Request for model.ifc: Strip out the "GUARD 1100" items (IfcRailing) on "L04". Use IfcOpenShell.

First a look at what the model holds.

```python
import ifcopenshell
import ifcopenshell.util.element

model = ifcopenshell.open("model.ifc")
print(model.schema)
storey = next(s for s in model.by_type("IfcBuildingStorey") if s.Name == "L04")
railings = [e for e in ifcopenshell.util.element.get_decomposition(storey) if e.is_a("IfcRailing")]
seen = {}
for e in railings:
    element_type = ifcopenshell.util.element.get_type(e)
    name = element_type.Name if element_type not in (None, e) else None
    seen[name] = seen.get(name, 0) + 1
for name, count in sorted(seen.items(), key=str):
    print(count, "x", name)
```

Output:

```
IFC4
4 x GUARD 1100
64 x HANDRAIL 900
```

```python
import ifcopenshell
import ifcopenshell.api.root
import ifcopenshell.util.element

model = ifcopenshell.open("model.ifc")

storey = next(s for s in model.by_type("IfcBuildingStorey") if s.Name == "L04")
railings = [e for e in ifcopenshell.util.element.get_decomposition(storey) if e.is_a("IfcRailing")]
targets = [e for e in railings if (t := ifcopenshell.util.element.get_type(e)) not in (None, e) and t.Name == "GUARD 1100"]

for e in targets:
    ifcopenshell.api.root.remove_product(model, product=e)
print(len(targets), "removed")

model.write("model-out.ifc")
```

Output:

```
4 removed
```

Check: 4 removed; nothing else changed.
